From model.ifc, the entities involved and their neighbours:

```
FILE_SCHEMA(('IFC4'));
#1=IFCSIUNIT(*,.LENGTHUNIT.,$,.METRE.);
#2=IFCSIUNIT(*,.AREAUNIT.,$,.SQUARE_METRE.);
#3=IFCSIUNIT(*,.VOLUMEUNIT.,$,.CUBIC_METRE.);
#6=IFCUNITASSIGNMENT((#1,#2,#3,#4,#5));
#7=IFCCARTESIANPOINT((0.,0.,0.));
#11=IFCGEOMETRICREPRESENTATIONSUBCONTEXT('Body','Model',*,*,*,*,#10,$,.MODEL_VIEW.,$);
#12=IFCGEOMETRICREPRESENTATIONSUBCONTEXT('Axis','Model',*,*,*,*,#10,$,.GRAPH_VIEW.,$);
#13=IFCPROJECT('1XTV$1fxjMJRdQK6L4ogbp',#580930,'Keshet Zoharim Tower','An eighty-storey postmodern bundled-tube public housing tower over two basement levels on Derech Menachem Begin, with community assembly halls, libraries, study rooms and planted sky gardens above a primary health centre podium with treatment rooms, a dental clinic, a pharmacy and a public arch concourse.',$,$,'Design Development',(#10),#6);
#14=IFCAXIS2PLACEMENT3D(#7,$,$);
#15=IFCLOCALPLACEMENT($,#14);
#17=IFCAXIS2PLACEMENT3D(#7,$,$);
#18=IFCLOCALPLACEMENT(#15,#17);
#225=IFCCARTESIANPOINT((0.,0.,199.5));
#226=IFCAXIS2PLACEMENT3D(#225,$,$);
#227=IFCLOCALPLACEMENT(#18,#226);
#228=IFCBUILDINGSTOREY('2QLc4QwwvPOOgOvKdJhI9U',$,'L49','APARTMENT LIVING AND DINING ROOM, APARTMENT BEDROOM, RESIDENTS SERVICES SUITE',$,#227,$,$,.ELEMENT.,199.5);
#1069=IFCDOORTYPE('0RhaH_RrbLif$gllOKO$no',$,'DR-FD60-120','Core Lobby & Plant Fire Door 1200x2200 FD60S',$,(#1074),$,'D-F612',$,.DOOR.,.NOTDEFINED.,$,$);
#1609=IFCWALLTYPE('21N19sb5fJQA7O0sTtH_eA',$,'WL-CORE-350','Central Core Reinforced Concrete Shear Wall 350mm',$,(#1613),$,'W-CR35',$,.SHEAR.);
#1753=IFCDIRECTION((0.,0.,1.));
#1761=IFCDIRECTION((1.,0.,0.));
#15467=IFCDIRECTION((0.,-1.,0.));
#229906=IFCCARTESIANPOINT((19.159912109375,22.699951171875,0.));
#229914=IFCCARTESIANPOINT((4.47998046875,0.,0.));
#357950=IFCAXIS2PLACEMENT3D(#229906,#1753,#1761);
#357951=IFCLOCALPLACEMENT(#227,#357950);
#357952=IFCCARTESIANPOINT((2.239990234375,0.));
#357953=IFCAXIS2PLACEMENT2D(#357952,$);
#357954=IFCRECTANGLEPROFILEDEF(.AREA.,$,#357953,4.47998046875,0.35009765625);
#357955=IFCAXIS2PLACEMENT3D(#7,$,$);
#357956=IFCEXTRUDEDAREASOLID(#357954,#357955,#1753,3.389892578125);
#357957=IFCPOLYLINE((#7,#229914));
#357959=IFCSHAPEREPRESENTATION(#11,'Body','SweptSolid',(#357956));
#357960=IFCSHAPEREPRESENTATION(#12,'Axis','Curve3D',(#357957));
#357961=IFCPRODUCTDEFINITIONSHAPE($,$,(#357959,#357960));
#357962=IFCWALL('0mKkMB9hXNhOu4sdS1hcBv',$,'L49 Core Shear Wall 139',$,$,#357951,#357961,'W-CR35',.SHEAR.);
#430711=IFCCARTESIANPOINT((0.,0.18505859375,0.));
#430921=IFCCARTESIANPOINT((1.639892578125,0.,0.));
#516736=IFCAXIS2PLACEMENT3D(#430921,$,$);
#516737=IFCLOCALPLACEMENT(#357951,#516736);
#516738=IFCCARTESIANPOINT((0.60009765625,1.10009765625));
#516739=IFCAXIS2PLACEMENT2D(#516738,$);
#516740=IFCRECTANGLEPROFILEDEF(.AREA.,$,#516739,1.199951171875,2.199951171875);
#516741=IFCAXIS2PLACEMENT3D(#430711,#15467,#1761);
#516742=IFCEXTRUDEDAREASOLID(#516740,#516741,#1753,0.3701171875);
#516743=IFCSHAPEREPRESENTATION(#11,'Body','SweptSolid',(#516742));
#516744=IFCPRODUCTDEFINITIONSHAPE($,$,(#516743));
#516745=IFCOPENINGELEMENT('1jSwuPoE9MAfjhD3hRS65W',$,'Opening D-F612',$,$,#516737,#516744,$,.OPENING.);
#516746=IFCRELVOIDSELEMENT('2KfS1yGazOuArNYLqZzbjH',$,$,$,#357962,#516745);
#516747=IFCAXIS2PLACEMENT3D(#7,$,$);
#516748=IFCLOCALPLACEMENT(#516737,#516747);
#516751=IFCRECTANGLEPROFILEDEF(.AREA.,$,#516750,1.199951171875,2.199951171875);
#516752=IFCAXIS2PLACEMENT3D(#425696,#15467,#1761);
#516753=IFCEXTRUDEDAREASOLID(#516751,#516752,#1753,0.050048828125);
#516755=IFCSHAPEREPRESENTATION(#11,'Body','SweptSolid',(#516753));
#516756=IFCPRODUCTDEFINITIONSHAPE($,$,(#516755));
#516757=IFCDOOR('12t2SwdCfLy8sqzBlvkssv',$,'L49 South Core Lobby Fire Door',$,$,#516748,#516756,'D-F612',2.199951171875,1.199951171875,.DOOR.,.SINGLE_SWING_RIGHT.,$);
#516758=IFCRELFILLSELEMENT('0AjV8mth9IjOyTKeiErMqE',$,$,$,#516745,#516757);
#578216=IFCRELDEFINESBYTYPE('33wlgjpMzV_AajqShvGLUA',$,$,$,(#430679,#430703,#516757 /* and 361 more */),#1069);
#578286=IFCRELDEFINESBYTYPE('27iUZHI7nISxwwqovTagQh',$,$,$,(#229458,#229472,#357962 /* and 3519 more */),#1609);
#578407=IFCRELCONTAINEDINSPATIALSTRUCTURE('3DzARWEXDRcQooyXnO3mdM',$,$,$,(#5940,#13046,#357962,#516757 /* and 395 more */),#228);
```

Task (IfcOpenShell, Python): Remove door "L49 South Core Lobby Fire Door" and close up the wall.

```python
import ifcopenshell
import ifcopenshell.api.feature
import ifcopenshell.api.root
import ifcopenshell.geom
import ifcopenshell.util.shape

model = ifcopenshell.open("model.ifc")
settings = ifcopenshell.geom.settings()


def volume(element):
    """Net volume in cubic metres, openings subtracted."""
    shape = ifcopenshell.geom.create_shape(settings, element)
    return ifcopenshell.util.shape.get_volume(shape.geometry)


door = model.by_guid("12t2SwdCfLy8sqzBlvkssv")
opening = door.FillsVoids[0].RelatingOpeningElement
wall = opening.VoidsElements[0].RelatingBuildingElement
before = volume(wall)

ifcopenshell.api.root.remove_product(model, product=door)
ifcopenshell.api.feature.remove_feature(model, feature=opening)

after = volume(wall)

print(f"wall volume {before:.3f} -> {after:.3f} m3")

model.write("model-out.ifc")
```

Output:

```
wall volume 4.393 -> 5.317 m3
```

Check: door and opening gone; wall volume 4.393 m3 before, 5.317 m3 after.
